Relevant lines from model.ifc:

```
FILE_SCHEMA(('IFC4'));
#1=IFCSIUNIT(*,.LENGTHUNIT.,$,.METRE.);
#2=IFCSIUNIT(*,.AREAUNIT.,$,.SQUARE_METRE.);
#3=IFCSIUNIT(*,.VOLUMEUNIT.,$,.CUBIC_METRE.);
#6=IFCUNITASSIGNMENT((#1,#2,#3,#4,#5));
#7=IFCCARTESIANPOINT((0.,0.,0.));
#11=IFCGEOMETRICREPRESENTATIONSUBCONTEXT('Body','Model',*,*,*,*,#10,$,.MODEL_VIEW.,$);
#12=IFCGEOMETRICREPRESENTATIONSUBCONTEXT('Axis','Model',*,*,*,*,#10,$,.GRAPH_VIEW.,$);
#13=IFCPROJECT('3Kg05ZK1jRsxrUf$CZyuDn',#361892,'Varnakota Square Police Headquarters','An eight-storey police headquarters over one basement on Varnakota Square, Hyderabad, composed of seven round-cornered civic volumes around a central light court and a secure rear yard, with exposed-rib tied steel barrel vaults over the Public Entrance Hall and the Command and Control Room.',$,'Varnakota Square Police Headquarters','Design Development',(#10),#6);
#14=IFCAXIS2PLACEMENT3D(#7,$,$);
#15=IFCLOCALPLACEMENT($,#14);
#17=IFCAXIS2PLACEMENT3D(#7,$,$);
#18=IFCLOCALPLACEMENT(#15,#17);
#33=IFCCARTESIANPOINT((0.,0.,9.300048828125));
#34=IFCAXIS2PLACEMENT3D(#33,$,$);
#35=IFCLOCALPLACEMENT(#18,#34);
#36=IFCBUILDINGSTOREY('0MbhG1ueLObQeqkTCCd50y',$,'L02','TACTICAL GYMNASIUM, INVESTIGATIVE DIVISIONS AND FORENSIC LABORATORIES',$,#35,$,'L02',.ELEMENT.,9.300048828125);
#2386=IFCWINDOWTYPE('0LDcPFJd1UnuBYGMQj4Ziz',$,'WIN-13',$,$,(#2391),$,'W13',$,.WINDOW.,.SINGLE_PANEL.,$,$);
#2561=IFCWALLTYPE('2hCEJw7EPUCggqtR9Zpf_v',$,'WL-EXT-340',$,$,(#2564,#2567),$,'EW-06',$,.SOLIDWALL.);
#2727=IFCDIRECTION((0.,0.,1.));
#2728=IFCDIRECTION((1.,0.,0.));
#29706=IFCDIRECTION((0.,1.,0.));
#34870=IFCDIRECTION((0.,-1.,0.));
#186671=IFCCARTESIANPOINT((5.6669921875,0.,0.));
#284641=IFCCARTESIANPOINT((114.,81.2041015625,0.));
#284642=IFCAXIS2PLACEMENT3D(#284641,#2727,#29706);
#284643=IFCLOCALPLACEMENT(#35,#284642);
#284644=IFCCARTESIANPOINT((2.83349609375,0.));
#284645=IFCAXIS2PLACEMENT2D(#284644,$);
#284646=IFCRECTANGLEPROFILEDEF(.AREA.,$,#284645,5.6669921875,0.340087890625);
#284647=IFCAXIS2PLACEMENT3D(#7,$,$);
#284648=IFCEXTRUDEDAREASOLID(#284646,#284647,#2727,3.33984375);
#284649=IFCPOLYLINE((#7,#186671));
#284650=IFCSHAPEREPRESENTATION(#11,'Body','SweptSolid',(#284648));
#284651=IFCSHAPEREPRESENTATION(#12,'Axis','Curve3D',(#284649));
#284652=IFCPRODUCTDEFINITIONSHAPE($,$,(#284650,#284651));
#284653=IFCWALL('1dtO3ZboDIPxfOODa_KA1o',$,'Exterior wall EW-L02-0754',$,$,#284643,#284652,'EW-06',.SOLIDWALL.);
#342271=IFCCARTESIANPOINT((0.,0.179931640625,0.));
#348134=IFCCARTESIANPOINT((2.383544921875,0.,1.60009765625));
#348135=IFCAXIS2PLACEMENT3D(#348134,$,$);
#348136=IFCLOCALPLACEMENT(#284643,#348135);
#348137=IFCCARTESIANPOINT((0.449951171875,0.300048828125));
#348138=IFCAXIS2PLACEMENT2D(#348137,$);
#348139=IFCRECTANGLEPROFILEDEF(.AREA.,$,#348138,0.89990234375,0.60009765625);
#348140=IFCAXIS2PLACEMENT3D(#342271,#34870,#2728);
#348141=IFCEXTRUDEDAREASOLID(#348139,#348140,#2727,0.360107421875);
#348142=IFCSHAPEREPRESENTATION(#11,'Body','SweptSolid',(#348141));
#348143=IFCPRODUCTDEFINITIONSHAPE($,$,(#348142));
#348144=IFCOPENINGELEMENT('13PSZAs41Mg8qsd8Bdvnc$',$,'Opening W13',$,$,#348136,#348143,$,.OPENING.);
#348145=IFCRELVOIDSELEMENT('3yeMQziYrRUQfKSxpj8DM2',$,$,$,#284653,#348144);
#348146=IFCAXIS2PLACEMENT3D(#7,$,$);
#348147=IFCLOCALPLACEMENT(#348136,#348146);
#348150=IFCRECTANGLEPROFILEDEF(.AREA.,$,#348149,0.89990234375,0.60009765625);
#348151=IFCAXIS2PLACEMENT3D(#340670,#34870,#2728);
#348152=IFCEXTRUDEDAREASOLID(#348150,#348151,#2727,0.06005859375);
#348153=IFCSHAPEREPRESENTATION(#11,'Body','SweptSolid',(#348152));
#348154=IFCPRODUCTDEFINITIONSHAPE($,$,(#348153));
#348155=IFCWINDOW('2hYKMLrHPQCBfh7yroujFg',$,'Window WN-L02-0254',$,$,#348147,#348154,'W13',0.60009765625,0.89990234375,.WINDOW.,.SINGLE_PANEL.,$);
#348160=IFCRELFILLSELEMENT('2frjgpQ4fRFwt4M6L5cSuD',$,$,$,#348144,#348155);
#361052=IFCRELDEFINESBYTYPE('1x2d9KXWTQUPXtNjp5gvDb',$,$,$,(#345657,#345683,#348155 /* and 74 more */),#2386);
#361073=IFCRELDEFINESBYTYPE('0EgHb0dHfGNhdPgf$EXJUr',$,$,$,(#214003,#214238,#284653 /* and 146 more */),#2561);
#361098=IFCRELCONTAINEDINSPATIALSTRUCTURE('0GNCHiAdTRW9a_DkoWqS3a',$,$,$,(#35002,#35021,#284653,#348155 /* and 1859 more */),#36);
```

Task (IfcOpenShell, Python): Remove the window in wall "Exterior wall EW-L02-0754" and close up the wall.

```python
import ifcopenshell
import ifcopenshell.api.feature
import ifcopenshell.api.root
import ifcopenshell.geom
import ifcopenshell.util.shape

model = ifcopenshell.open("model.ifc")
settings = ifcopenshell.geom.settings()


def volume(element):
    """Net volume in cubic metres, openings subtracted."""
    shape = ifcopenshell.geom.create_shape(settings, element)
    return ifcopenshell.util.shape.get_volume(shape.geometry)


window = model.by_guid("2hYKMLrHPQCBfh7yroujFg")
opening = window.FillsVoids[0].RelatingOpeningElement
wall = opening.VoidsElements[0].RelatingBuildingElement
before = volume(wall)

ifcopenshell.api.root.remove_product(model, product=window)
ifcopenshell.api.feature.remove_feature(model, feature=opening)

after = volume(wall)

print(f"wall volume {before:.3f} -> {after:.3f} m3")

model.write("model_rev.ifc")
```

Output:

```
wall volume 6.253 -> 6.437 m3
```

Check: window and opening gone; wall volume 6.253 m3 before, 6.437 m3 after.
